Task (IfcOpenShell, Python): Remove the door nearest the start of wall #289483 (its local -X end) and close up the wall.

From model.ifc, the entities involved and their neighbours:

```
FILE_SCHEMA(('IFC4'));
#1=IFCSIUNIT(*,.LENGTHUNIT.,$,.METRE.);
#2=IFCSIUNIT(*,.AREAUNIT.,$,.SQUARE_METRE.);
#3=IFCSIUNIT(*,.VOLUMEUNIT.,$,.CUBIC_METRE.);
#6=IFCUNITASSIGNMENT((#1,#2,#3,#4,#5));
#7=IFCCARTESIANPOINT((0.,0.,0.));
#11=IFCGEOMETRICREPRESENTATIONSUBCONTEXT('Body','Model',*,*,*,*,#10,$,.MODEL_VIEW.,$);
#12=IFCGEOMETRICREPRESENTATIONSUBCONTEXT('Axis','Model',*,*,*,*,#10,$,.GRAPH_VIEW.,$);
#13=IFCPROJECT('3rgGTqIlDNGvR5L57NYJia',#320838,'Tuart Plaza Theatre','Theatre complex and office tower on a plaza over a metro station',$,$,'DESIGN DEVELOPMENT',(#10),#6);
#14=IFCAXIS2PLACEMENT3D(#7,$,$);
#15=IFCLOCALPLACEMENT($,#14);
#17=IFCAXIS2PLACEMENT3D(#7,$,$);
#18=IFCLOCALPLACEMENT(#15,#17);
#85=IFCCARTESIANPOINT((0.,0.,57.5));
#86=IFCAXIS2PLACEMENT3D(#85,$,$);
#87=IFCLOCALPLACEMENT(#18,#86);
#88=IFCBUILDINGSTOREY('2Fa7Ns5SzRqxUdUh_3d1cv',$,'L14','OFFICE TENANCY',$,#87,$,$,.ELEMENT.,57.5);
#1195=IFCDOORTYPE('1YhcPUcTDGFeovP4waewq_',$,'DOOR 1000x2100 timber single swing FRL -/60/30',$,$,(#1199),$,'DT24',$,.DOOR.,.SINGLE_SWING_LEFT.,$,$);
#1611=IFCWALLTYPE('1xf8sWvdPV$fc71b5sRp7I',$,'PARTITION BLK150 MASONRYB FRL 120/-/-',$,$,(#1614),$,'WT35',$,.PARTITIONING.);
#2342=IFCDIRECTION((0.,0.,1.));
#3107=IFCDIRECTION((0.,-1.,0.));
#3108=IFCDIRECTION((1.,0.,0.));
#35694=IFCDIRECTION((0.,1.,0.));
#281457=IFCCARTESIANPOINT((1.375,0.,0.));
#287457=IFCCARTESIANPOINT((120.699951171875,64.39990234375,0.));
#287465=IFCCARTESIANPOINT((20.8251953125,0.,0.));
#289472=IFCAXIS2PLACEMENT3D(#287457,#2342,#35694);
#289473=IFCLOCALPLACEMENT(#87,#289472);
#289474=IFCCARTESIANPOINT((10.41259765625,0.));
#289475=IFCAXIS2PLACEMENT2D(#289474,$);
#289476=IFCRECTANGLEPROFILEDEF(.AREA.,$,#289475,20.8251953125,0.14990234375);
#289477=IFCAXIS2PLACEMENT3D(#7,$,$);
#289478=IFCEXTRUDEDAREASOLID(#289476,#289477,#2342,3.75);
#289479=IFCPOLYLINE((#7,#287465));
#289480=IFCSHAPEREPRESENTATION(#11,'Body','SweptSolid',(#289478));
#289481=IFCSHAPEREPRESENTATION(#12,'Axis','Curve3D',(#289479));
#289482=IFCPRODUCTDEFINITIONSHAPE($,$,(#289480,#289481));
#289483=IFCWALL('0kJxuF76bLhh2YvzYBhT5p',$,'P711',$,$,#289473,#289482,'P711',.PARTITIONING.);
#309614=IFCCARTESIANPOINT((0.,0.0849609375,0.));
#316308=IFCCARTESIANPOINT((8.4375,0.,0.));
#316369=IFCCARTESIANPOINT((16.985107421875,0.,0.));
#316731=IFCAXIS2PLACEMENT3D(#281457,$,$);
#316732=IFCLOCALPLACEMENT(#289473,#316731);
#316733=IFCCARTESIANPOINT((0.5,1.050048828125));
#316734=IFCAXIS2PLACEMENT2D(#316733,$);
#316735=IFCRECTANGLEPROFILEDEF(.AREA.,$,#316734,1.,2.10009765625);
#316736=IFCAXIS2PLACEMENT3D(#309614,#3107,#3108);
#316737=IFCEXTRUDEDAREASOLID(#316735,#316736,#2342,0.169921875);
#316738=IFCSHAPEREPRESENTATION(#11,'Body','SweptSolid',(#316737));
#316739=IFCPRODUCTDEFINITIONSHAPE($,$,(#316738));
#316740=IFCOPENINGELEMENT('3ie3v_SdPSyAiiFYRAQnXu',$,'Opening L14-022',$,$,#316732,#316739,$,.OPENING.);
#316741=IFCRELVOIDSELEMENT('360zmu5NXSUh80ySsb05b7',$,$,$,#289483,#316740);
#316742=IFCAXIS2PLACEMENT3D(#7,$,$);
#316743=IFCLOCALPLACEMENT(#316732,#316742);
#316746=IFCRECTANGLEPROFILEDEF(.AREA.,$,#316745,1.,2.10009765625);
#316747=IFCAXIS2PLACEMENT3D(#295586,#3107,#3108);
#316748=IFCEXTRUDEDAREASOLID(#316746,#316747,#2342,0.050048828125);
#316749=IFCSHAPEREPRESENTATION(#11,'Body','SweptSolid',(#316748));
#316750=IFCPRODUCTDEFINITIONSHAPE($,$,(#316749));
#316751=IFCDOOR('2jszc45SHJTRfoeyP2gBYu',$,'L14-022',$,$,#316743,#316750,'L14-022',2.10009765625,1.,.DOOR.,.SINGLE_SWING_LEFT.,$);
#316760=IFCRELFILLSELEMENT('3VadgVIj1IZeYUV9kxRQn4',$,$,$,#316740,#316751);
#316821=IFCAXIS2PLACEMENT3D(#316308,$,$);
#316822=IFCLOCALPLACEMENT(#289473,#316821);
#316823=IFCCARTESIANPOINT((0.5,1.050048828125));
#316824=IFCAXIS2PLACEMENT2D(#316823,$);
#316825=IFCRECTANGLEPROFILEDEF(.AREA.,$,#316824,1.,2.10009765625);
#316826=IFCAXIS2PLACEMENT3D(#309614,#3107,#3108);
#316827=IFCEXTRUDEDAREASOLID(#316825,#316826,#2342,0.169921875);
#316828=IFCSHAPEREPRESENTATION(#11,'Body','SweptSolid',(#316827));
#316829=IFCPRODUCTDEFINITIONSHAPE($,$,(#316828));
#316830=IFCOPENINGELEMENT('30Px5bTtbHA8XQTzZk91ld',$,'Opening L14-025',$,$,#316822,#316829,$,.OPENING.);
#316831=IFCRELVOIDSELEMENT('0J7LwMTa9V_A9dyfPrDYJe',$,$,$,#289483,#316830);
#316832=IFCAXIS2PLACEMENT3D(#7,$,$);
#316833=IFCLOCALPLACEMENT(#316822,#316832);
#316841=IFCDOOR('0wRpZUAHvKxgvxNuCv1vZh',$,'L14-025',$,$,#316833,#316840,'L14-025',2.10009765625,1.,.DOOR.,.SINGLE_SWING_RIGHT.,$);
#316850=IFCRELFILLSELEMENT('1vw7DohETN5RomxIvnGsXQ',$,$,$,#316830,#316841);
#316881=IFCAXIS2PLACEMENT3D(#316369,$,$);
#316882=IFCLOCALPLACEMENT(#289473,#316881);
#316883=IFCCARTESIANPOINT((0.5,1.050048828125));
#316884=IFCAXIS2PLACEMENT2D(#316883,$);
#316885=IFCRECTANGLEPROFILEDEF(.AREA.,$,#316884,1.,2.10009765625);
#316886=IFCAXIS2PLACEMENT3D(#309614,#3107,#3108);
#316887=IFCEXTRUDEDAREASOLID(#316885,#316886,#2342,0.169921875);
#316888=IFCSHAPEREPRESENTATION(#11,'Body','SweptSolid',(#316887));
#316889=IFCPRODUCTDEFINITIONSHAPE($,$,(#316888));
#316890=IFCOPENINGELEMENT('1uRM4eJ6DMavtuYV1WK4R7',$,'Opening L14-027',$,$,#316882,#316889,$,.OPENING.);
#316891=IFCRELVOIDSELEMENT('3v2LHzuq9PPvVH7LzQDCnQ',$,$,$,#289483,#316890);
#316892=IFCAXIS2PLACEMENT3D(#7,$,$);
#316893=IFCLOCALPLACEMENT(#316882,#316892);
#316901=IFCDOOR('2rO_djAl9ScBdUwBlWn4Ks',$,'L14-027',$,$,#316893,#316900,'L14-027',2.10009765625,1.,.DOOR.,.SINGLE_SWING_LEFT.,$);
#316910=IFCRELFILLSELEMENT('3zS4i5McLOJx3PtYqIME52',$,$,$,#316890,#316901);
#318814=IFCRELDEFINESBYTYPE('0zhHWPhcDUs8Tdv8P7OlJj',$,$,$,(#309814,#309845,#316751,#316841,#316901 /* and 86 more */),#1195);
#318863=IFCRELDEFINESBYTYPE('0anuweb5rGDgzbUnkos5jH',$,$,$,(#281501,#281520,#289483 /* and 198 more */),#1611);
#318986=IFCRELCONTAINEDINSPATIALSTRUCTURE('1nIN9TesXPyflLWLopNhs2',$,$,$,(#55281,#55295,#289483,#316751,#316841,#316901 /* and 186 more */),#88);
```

```python
import ifcopenshell
import ifcopenshell.api.feature
import ifcopenshell.api.root
import ifcopenshell.geom
import ifcopenshell.util.shape

model = ifcopenshell.open("model.ifc")
settings = ifcopenshell.geom.settings()


def volume(element):
    """Net volume in cubic metres, openings subtracted."""
    shape = ifcopenshell.geom.create_shape(settings, element)
    return ifcopenshell.util.shape.get_volume(shape.geometry)


door = model.by_guid("2jszc45SHJTRfoeyP2gBYu")
opening = door.FillsVoids[0].RelatingOpeningElement
wall = opening.VoidsElements[0].RelatingBuildingElement
before = volume(wall)

ifcopenshell.api.root.remove_product(model, product=door)
ifcopenshell.api.feature.remove_feature(model, feature=opening)

after = volume(wall)

print(f"wall volume {before:.3f} -> {after:.3f} m3")

model.write("model_updated.ifc")
```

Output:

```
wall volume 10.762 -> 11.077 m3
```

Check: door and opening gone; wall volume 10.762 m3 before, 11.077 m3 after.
